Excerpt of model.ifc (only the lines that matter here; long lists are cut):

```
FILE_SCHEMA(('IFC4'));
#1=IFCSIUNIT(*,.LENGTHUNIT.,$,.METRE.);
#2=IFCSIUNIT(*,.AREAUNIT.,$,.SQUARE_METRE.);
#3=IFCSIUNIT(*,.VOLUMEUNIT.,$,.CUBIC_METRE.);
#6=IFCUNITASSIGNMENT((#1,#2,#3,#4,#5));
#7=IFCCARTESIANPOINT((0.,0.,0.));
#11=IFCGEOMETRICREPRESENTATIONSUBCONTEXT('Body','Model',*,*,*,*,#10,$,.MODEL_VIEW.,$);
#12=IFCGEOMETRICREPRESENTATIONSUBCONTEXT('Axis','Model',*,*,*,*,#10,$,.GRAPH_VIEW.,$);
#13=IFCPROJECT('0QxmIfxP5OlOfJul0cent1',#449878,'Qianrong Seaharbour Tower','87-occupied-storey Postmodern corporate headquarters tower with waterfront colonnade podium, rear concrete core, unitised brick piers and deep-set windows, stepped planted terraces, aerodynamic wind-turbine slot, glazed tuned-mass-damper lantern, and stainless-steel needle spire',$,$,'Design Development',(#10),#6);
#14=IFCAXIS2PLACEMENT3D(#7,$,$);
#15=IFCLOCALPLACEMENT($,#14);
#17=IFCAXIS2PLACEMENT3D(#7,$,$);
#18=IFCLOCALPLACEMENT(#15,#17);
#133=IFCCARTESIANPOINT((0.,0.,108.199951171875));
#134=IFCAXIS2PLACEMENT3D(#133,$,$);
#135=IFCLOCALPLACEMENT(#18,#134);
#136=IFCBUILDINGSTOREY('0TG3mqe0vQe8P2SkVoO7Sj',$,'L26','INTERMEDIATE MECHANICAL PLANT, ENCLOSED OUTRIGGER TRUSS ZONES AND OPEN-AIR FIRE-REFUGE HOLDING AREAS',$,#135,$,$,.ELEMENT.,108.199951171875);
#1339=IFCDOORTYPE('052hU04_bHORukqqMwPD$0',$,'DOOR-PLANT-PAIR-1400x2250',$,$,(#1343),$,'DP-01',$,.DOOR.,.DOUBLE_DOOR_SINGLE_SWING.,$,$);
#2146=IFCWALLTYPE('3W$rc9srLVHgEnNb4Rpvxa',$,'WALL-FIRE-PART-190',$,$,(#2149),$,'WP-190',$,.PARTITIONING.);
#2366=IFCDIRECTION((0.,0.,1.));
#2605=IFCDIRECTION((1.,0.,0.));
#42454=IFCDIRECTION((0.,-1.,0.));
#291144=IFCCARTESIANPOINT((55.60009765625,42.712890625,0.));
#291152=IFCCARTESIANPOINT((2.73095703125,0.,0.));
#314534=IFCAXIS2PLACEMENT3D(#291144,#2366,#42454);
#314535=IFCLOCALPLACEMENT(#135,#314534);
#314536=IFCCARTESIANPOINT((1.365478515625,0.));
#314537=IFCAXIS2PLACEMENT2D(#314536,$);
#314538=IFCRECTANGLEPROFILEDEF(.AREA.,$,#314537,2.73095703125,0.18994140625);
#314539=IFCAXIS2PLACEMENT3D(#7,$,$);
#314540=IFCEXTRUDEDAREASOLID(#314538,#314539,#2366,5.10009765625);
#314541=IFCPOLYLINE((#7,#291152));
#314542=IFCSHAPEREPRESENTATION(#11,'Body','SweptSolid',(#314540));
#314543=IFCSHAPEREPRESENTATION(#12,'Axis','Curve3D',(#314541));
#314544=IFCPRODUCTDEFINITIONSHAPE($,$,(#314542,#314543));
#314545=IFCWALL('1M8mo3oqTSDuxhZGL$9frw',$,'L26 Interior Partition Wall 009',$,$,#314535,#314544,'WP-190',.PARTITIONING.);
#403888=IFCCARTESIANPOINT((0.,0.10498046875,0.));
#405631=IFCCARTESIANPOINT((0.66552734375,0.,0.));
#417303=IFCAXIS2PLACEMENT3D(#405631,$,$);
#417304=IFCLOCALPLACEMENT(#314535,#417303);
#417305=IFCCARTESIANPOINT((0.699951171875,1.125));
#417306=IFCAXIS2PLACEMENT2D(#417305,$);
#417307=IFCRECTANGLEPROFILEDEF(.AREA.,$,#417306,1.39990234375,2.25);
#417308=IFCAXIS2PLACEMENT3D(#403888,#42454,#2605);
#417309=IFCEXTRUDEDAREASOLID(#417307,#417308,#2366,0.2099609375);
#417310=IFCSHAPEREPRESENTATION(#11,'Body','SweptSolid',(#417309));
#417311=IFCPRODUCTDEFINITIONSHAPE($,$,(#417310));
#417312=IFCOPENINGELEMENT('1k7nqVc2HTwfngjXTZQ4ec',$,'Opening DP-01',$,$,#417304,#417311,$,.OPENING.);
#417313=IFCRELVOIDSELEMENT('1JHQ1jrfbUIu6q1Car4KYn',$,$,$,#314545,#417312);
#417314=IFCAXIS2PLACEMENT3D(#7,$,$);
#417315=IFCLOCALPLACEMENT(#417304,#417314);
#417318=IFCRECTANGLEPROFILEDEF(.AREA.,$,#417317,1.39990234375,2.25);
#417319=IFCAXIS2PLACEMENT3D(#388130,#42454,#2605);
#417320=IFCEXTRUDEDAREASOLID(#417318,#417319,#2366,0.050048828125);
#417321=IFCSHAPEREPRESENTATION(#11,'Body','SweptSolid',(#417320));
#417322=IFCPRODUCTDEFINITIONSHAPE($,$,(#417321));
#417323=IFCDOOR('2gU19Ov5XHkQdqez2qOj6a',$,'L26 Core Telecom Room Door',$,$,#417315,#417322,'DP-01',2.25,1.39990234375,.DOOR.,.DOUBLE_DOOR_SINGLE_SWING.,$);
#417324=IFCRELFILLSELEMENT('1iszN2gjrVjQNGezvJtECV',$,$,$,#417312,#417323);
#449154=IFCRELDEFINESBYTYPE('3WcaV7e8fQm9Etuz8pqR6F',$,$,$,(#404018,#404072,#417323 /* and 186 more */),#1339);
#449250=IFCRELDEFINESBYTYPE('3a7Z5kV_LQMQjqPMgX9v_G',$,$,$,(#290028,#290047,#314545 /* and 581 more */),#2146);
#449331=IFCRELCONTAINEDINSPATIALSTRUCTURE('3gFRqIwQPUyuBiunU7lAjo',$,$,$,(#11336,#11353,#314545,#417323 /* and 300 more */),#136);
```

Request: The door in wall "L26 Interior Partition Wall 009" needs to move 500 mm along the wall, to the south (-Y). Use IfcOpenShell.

```python
import ifcopenshell
import ifcopenshell.api.geometry
import ifcopenshell.util.placement
import ifcopenshell.util.unit

model = ifcopenshell.open("model.ifc")
unit_scale = ifcopenshell.util.unit.calculate_unit_scale(model)

door = model.by_guid("2gU19Ov5XHkQdqez2qOj6a")
opening = door.FillsVoids[0].RelatingOpeningElement
wall = opening.VoidsElements[0].RelatingBuildingElement

wall_matrix = ifcopenshell.util.placement.get_local_placement(wall.ObjectPlacement)
shift = wall_matrix[:3, 0] * 0.5 / unit_scale
before = ifcopenshell.util.placement.get_local_placement(door.ObjectPlacement)[:3, 3].copy()

# The door is placed relative to its opening, so it follows when the opening moves.
matrix = ifcopenshell.util.placement.get_local_placement(opening.ObjectPlacement)
matrix[:3, 3] += shift
ifcopenshell.api.geometry.edit_object_placement(
    model, product=opening, matrix=matrix, is_si=False, should_transform_children=True
)

after = ifcopenshell.util.placement.get_local_placement(door.ObjectPlacement)[:3, 3]
print("door moved by", (after - before).round(3) + 0.0)

model.write("model_edited.ifc")
```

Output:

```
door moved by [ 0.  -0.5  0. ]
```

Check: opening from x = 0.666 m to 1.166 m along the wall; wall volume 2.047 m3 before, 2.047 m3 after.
